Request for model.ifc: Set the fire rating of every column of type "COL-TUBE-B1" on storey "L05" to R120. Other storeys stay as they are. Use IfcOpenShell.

First a look at what the model holds.

```python
import ifcopenshell
import ifcopenshell.util.element

model = ifcopenshell.open("model.ifc")
print(model.schema)
storey = next(s for s in model.by_type("IfcBuildingStorey") if s.Name == "L05")
columns = [e for e in ifcopenshell.util.element.get_decomposition(storey) if e.is_a("IfcColumn")]
seen = {}
for e in columns:
    element_type = ifcopenshell.util.element.get_type(e)
    key = (element_type.Name if element_type != e and element_type else None, ifcopenshell.util.element.get_pset(e, "Pset_ColumnCommon", "FireRating"))
    seen[key] = seen.get(key, 0) + 1
for (name, value), count in sorted(seen.items(), key=str):
    print(count, "x", name, "|", value)
```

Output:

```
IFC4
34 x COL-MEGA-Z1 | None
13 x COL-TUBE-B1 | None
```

```python
import ifcopenshell
import ifcopenshell.api.pset
import ifcopenshell.util.element

model = ifcopenshell.open("model.ifc")

storey = next(s for s in model.by_type("IfcBuildingStorey") if s.Name == "L05")
columns = [e for e in ifcopenshell.util.element.get_decomposition(storey) if e.is_a("IfcColumn")]

count = 0
for e in columns:
    element_type = ifcopenshell.util.element.get_type(e)
    if element_type in (None, e) or element_type.Name != "COL-TUBE-B1":
        continue
    found = ifcopenshell.util.element.get_pset(e, "Pset_ColumnCommon", should_inherit=False)
    if found:
        pset = model.by_id(found["id"])
        if len(ifcopenshell.util.element.get_elements_by_pset(pset)) > 1:
            pset = ifcopenshell.api.pset.unshare_pset(model, products=[e], pset=pset)[0]
    else:
        pset = ifcopenshell.api.pset.add_pset(model, product=e, name="Pset_ColumnCommon")
    ifcopenshell.api.pset.edit_pset(model, pset=pset, properties={"FireRating": "R120"})
    count += 1

print(count, "columns updated")

model.write("model_edited.ifc")
```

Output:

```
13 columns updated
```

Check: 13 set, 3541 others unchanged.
